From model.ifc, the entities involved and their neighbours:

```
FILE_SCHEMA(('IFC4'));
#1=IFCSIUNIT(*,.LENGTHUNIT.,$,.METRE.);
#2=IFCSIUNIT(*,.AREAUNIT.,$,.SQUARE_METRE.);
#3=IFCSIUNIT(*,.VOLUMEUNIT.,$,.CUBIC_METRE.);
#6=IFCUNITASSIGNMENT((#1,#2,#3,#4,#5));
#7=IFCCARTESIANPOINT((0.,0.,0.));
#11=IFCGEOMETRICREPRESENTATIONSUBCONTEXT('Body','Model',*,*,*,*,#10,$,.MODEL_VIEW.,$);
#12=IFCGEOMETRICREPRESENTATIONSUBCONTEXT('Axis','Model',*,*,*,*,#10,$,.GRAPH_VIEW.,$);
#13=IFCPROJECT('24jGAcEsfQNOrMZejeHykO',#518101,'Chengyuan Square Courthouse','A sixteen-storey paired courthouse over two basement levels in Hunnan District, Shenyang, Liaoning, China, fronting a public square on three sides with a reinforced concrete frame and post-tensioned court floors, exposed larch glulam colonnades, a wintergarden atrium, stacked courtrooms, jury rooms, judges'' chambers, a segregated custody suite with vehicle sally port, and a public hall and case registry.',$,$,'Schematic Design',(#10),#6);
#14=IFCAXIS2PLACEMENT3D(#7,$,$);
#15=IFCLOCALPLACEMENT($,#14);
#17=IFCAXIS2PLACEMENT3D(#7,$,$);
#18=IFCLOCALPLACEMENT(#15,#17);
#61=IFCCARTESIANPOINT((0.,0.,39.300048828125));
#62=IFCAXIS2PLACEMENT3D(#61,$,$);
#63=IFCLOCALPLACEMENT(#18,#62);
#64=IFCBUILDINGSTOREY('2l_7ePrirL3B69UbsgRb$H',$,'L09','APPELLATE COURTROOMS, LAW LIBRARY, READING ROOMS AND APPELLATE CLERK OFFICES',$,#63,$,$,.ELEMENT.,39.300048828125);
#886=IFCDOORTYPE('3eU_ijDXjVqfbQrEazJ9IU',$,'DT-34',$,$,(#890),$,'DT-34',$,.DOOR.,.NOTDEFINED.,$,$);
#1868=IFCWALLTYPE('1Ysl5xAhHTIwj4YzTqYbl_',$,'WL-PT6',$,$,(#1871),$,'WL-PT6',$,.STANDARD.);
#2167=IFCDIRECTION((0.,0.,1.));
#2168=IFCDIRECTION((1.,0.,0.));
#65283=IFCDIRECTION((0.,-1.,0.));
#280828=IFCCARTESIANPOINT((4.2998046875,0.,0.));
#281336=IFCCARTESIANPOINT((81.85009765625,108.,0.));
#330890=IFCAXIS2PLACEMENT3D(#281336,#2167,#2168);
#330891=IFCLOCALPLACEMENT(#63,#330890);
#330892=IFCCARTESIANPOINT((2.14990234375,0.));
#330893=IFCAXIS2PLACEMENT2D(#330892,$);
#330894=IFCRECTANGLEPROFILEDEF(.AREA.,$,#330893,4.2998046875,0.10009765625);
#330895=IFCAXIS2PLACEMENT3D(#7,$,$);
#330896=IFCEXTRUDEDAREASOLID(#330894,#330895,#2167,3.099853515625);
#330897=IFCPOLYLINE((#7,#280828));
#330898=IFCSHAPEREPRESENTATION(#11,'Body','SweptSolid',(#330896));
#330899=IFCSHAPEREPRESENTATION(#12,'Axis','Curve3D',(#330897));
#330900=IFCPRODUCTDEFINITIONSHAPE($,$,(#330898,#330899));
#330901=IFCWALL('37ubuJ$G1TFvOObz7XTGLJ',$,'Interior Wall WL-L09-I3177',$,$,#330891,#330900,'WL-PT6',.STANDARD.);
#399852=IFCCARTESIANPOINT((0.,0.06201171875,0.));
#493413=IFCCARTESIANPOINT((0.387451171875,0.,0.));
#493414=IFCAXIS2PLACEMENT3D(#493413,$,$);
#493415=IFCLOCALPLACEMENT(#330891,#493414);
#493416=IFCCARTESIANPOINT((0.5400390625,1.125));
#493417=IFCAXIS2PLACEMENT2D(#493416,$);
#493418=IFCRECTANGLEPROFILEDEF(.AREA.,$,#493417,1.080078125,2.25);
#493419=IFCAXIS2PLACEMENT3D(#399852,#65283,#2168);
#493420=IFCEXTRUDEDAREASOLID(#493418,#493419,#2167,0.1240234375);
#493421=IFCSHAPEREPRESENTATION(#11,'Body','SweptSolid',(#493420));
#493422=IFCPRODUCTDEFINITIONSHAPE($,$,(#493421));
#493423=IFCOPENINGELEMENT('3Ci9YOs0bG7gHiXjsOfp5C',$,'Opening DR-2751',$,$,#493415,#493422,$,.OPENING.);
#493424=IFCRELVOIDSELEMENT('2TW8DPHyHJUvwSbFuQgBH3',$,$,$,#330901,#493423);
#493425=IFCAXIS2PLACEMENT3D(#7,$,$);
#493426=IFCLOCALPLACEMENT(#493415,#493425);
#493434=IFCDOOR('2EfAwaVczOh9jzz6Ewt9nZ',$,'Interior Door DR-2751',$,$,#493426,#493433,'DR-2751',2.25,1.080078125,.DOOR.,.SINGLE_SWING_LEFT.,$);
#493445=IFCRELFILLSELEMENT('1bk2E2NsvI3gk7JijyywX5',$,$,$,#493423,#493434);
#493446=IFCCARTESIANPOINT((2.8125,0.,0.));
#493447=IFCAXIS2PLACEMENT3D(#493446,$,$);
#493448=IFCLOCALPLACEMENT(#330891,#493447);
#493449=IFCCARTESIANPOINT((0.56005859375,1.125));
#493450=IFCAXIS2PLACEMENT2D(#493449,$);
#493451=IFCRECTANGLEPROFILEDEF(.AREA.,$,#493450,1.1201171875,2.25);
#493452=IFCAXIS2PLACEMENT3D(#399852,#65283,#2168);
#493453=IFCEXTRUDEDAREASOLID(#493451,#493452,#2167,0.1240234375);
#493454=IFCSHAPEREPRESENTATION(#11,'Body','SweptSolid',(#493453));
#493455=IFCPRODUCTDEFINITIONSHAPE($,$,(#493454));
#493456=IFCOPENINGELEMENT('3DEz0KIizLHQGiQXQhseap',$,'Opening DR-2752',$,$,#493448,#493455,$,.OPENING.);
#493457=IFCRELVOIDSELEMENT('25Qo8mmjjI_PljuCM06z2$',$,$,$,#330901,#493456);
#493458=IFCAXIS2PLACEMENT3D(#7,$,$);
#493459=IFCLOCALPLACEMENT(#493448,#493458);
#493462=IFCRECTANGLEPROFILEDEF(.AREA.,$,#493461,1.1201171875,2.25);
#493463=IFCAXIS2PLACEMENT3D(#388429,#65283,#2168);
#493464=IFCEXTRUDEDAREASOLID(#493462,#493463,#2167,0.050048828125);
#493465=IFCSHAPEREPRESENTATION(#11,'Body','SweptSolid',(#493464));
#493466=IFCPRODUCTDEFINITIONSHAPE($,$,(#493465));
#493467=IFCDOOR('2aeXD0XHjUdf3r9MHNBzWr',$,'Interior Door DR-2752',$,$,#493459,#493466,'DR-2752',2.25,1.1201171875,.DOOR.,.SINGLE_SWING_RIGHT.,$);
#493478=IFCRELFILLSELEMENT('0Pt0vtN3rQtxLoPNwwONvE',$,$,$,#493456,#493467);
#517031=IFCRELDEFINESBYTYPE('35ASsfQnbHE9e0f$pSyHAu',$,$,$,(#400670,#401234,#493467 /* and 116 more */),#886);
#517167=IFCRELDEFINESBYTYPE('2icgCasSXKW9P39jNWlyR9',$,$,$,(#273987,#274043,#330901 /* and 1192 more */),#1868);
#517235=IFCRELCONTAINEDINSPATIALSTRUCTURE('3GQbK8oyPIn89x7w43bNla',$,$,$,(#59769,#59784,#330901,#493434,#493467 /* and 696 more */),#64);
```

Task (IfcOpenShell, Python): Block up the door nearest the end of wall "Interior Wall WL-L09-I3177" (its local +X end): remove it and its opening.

```python
import ifcopenshell
import ifcopenshell.api.feature
import ifcopenshell.api.root
import ifcopenshell.geom
import ifcopenshell.util.shape

model = ifcopenshell.open("model.ifc")
settings = ifcopenshell.geom.settings()


def volume(element):
    """Net volume in cubic metres, openings subtracted."""
    shape = ifcopenshell.geom.create_shape(settings, element)
    return ifcopenshell.util.shape.get_volume(shape.geometry)


door = model.by_guid("2aeXD0XHjUdf3r9MHNBzWr")
opening = door.FillsVoids[0].RelatingOpeningElement
wall = opening.VoidsElements[0].RelatingBuildingElement
before = volume(wall)

ifcopenshell.api.root.remove_product(model, product=door)
ifcopenshell.api.feature.remove_feature(model, feature=opening)

after = volume(wall)

print(f"wall volume {before:.3f} -> {after:.3f} m3")

model.write("model_edited.ifc")
```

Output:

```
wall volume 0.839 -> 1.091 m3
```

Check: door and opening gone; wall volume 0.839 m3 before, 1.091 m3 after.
